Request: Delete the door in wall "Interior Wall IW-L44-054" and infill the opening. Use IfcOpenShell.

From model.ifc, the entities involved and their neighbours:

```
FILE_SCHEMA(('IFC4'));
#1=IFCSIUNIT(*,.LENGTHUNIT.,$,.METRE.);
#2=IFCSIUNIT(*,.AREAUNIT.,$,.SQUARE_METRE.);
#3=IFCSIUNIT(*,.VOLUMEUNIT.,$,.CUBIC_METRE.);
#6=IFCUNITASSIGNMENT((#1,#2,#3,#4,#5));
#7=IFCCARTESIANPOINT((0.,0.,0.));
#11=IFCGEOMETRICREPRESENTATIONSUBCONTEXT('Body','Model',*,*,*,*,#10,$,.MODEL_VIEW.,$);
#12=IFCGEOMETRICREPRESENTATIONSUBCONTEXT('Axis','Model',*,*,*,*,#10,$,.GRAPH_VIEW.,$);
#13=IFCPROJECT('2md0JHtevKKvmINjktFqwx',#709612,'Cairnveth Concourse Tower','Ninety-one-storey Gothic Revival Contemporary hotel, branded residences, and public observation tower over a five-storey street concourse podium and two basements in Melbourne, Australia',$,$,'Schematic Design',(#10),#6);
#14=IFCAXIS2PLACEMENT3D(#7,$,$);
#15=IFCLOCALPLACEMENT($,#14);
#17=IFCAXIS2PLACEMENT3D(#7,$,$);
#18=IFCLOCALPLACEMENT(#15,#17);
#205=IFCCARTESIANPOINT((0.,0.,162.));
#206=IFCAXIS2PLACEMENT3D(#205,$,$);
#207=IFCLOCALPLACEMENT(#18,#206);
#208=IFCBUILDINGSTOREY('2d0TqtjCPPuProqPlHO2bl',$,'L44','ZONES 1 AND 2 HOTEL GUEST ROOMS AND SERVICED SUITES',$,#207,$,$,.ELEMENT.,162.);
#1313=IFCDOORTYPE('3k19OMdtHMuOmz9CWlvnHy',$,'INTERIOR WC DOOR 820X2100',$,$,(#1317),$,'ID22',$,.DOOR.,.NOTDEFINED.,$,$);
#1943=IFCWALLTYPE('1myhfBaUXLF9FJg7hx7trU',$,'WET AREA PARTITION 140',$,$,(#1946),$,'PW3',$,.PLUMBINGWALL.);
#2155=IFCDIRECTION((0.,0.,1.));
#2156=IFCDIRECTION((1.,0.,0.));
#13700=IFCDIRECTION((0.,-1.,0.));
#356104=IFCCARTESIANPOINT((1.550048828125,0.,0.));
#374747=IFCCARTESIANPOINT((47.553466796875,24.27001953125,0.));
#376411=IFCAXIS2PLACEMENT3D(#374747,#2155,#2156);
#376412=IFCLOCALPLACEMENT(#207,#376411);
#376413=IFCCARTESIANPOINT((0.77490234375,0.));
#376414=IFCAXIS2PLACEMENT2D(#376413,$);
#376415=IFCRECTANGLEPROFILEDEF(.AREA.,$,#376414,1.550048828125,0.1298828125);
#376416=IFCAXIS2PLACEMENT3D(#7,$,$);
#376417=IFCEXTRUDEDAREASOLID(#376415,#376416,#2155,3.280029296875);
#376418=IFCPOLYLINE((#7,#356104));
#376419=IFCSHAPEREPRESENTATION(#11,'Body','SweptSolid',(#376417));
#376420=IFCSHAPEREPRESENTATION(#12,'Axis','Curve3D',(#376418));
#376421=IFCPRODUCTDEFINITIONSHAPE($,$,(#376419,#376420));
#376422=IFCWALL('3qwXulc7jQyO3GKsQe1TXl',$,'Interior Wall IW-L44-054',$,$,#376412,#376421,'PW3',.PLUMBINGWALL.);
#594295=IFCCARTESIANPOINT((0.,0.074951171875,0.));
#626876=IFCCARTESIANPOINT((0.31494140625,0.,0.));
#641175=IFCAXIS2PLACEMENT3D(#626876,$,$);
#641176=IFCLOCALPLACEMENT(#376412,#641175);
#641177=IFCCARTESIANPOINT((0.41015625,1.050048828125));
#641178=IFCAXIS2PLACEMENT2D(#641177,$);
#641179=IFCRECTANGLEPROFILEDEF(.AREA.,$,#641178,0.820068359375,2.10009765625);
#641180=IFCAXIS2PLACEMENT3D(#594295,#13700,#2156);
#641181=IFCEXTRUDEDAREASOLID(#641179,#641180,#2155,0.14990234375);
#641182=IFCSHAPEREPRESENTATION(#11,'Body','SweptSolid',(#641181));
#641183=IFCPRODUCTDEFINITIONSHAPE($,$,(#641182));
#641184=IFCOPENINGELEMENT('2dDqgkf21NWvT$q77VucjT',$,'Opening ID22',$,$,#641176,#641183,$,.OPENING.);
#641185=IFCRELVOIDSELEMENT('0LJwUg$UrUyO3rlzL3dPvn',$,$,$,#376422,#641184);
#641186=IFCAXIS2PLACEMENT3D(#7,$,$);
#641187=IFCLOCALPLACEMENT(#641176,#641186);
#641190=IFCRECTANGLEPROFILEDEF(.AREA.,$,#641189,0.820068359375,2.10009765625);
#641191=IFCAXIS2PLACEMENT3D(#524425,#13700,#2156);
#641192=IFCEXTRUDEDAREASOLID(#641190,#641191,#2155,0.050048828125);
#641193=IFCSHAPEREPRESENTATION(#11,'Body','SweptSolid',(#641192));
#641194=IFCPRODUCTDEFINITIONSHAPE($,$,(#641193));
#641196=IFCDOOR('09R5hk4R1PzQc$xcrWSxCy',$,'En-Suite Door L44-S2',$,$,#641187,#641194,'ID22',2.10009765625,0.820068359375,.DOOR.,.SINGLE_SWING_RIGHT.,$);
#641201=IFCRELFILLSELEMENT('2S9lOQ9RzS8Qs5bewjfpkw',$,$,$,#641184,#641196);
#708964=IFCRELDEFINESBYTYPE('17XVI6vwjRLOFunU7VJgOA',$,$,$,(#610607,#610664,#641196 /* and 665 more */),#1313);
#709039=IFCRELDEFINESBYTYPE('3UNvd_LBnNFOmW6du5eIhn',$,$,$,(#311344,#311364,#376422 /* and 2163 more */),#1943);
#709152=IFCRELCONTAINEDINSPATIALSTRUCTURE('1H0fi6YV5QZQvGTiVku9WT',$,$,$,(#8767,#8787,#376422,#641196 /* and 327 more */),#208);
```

```python
import ifcopenshell
import ifcopenshell.api.feature
import ifcopenshell.api.root
import ifcopenshell.geom
import ifcopenshell.util.shape

model = ifcopenshell.open("model.ifc")
settings = ifcopenshell.geom.settings()


def volume(element):
    """Net volume in cubic metres, openings subtracted."""
    shape = ifcopenshell.geom.create_shape(settings, element)
    return ifcopenshell.util.shape.get_volume(shape.geometry)


door = model.by_id(641196)
opening = door.FillsVoids[0].RelatingOpeningElement
wall = opening.VoidsElements[0].RelatingBuildingElement
before = volume(wall)

ifcopenshell.api.root.remove_product(model, product=door)
ifcopenshell.api.feature.remove_feature(model, feature=opening)

after = volume(wall)

print(f"wall volume {before:.3f} -> {after:.3f} m3")

model.write("model_v2.ifc")
```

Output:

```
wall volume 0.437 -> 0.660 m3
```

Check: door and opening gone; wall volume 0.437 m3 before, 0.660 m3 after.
